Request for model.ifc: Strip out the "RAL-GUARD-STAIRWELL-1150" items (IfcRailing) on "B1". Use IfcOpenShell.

First a look at what the model holds.

```python
import ifcopenshell
import ifcopenshell.util.element

model = ifcopenshell.open("model.ifc")
print(model.schema)
storey = next(s for s in model.by_type("IfcBuildingStorey") if s.Name == "B1")
railings = [e for e in ifcopenshell.util.element.get_decomposition(storey) if e.is_a("IfcRailing")]
seen = {}
for e in railings:
    element_type = ifcopenshell.util.element.get_type(e)
    name = element_type.Name if element_type not in (None, e) else None
    seen[name] = seen.get(name, 0) + 1
for name, count in sorted(seen.items(), key=str):
    print(count, "x", name)
```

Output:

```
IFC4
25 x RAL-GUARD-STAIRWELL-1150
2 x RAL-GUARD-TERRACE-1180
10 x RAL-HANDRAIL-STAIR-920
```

```python
import ifcopenshell
import ifcopenshell.api.root
import ifcopenshell.util.element

model = ifcopenshell.open("model.ifc")

storey = next(s for s in model.by_type("IfcBuildingStorey") if s.Name == "B1")
railings = [e for e in ifcopenshell.util.element.get_decomposition(storey) if e.is_a("IfcRailing")]
targets = [e for e in railings if (t := ifcopenshell.util.element.get_type(e)) not in (None, e) and t.Name == "RAL-GUARD-STAIRWELL-1150"]

for e in targets:
    ifcopenshell.api.root.remove_product(model, product=e)
print(len(targets), "removed")

model.write("model-out.ifc")
```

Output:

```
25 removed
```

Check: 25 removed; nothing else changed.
